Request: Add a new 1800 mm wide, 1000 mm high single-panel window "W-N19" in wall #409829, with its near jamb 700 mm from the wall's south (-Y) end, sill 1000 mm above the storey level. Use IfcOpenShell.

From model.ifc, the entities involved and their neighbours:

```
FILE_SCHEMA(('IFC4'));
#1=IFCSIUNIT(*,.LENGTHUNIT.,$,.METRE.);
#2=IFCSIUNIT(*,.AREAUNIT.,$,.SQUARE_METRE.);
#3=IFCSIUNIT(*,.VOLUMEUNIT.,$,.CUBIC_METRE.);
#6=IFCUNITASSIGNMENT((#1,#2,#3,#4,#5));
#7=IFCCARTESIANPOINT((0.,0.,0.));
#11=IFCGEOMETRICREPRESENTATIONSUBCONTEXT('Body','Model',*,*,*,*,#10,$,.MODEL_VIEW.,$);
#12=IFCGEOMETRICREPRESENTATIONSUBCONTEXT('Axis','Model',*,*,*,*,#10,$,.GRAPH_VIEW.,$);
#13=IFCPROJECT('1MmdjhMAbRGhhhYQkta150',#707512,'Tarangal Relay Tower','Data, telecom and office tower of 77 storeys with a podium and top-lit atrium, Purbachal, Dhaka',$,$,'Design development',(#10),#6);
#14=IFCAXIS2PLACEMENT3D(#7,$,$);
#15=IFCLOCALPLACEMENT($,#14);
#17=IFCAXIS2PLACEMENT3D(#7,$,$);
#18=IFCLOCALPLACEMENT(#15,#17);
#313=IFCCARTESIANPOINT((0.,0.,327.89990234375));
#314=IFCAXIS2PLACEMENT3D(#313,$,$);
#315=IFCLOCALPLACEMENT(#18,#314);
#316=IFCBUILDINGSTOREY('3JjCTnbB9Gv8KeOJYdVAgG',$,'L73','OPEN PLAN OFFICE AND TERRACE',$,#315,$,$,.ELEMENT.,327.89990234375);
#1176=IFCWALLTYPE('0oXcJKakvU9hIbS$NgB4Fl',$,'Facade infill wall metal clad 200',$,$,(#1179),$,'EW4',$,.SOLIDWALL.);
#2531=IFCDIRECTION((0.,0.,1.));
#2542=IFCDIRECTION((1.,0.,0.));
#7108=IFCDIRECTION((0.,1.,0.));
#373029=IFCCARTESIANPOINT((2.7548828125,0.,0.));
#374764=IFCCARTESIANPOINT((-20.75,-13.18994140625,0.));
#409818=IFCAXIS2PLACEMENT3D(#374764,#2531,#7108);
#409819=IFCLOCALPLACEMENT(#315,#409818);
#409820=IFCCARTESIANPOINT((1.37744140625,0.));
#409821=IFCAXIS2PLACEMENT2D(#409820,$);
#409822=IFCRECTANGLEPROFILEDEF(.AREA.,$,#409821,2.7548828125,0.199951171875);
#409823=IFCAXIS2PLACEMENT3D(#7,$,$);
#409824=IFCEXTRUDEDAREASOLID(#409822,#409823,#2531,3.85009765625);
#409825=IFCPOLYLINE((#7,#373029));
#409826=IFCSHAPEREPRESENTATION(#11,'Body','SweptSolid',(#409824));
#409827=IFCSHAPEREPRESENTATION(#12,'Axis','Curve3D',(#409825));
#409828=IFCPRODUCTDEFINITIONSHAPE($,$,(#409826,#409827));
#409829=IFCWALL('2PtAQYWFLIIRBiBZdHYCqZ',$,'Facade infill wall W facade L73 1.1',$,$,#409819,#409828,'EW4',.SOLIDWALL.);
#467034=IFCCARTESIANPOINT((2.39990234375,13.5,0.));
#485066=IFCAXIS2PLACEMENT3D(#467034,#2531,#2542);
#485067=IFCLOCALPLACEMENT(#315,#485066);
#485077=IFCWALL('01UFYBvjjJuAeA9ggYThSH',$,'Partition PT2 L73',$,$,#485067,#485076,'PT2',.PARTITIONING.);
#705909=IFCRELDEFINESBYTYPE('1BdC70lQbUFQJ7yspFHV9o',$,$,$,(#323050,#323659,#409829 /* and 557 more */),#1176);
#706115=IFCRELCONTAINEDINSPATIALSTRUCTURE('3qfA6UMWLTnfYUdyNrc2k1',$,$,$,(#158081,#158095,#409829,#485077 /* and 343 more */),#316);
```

```python
import numpy as np
import ifcopenshell
import ifcopenshell.api.feature
import ifcopenshell.api.geometry
import ifcopenshell.api.root
import ifcopenshell.api.spatial
import ifcopenshell.geom
import ifcopenshell.util.element
import ifcopenshell.util.placement
import ifcopenshell.util.representation
import ifcopenshell.util.shape
import ifcopenshell.util.unit

model = ifcopenshell.open("model.ifc")
unit_scale = ifcopenshell.util.unit.calculate_unit_scale(model)
settings = ifcopenshell.geom.settings()


def volume(element):
    """Net volume in cubic metres, openings subtracted."""
    shape = ifcopenshell.geom.create_shape(settings, element)
    return ifcopenshell.util.shape.get_volume(shape.geometry)


wall = model.by_id(409829)
storey = ifcopenshell.util.element.get_container(wall, ifc_class="IfcBuildingStorey")
context = ifcopenshell.util.representation.get_context(model, "Model", "Body", "MODEL_VIEW")
before = volume(wall)

width, height, from_end, sill = 1.8, 1, 0.7, 1  # metres

# The wall runs along its own X axis, and the end named is its -X end.
wall_shape = ifcopenshell.geom.create_shape(settings, wall)
x, y, z = ifcopenshell.util.shape.get_vertices(wall_shape.geometry).T
start = x.min() + from_end
face, thickness = float(y.min()), float(y.max() - y.min())
wall_matrix = ifcopenshell.util.placement.get_local_placement(wall.ObjectPlacement)
level = ifcopenshell.util.placement.get_local_placement(storey.ObjectPlacement)[2, 3]


def in_wall(x, y):
    """Placement at x, y metres in the wall's axes, at sill height."""
    matrix = wall_matrix.copy()
    matrix[:, 3] = wall_matrix @ np.array([x / unit_scale, y / unit_scale, 0.0, 1.0])
    matrix[2, 3] = level + sill / unit_scale
    return matrix


# Opening: a box that overshoots both wall faces by 50 mm.
opening = ifcopenshell.api.root.create_entity(model, ifc_class="IfcOpeningElement", predefined_type="OPENING")
box = ifcopenshell.api.geometry.add_wall_representation(
    model, context=context, length=width, height=height, thickness=thickness + 0.1
)
ifcopenshell.api.geometry.assign_representation(model, product=opening, representation=box)
ifcopenshell.api.geometry.edit_object_placement(model, product=opening, matrix=in_wall(start, face - 0.05), is_si=False)
ifcopenshell.api.feature.add_feature(model, feature=opening, element=wall)

window = ifcopenshell.api.root.create_entity(model, ifc_class="IfcWindow", name="W-N19", predefined_type="WINDOW")
window.OverallWidth, window.OverallHeight = width / unit_scale, height / unit_scale
window.PartitioningType = "SINGLE_PANEL"
body = ifcopenshell.api.geometry.add_window_representation(
    model,
    context=context,
    overall_width=window.OverallWidth,
    overall_height=window.OverallHeight,
    partition_type="SINGLE_PANEL",
)
ifcopenshell.api.geometry.assign_representation(model, product=window, representation=body)
ifcopenshell.api.spatial.assign_container(model, products=[window], relating_structure=storey)
ifcopenshell.api.feature.add_filling(model, opening=opening, element=window)

# Centre the window in the wall's thickness.
ifcopenshell.api.geometry.edit_object_placement(model, product=window, matrix=in_wall(start, face), is_si=False)
window_shape = ifcopenshell.geom.create_shape(settings, window)
depth = ifcopenshell.util.shape.get_vertices(window_shape.geometry)[:, 1]
offset = face + thickness / 2 - (depth.min() + depth.max()) / 2
ifcopenshell.api.geometry.edit_object_placement(model, product=window, matrix=in_wall(start, offset), is_si=False)

after = volume(wall)

print(f"wall volume {before:.3f} -> {after:.3f} m3")

model.write("model_rev.ifc")
```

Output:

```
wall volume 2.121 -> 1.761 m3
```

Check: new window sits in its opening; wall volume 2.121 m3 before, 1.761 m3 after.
